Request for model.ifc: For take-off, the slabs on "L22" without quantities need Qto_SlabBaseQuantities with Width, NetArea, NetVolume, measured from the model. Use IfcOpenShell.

First a look at what the model holds.

```python
import ifcopenshell
import ifcopenshell.util.element
import ifcopenshell.util.unit

model = ifcopenshell.open("model.ifc")
print(model.schema)
for unit_type in ("LENGTHUNIT", "AREAUNIT", "VOLUMEUNIT"):
    print(unit_type, ifcopenshell.util.unit.calculate_unit_scale(model, unit_type))
storey = next(s for s in model.by_type("IfcBuildingStorey") if s.Name == "L22")
slabs = [e for e in ifcopenshell.util.element.get_decomposition(storey) if e.is_a("IfcSlab")]
for e in sorted(slabs, key=lambda e: e.id()):
    print(e.id(), e.is_a(), e.Name, list(ifcopenshell.util.element.get_psets(e, qtos_only=True)), sep=" | ")
```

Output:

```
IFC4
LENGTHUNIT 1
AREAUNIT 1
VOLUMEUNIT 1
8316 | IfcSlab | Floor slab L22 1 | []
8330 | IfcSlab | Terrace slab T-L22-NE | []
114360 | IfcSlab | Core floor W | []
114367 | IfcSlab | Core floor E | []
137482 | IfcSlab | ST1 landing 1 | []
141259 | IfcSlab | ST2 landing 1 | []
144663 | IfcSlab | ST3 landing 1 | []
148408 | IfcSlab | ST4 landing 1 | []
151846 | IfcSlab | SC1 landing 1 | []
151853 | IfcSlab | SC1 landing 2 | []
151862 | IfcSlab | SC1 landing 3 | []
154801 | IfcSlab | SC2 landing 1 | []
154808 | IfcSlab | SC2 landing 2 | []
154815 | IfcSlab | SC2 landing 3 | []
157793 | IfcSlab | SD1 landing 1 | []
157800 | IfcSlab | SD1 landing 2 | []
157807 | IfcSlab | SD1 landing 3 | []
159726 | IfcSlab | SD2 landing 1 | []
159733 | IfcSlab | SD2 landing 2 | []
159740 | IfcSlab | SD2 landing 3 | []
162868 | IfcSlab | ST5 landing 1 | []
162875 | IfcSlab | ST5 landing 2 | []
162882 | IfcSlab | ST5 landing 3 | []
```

```python
import ifcopenshell
import ifcopenshell.api.pset
import ifcopenshell.geom
import ifcopenshell.util.element
import ifcopenshell.util.shape
import ifcopenshell.util.unit

model = ifcopenshell.open("model.ifc")
unit_scale = ifcopenshell.util.unit.calculate_unit_scale(model)
area_scale = ifcopenshell.util.unit.calculate_unit_scale(model, "AREAUNIT")
volume_scale = ifcopenshell.util.unit.calculate_unit_scale(model, "VOLUMEUNIT")
settings = ifcopenshell.geom.settings()

storey = next(s for s in model.by_type("IfcBuildingStorey") if s.Name == "L22")
slabs = [e for e in ifcopenshell.util.element.get_decomposition(storey) if e.is_a("IfcSlab")]

for e in sorted(slabs, key=lambda e: e.id()):
    if ifcopenshell.util.element.get_psets(e, qtos_only=True, should_inherit=False):
        continue
    # Geometry comes back in metres, in the element's own axes.
    shape = ifcopenshell.geom.create_shape(settings, e)
    values = {
        "Width": ifcopenshell.util.shape.get_z(shape.geometry) / unit_scale,
        "NetArea": ifcopenshell.util.shape.get_footprint_area(shape.geometry) / area_scale,
        "NetVolume": ifcopenshell.util.shape.get_volume(shape.geometry) / volume_scale,
    }
    qto = ifcopenshell.api.pset.add_qto(model, product=e, name="Qto_SlabBaseQuantities")
    ifcopenshell.api.pset.edit_qto(model, qto=qto, properties=values)
    print(e.id(), {k: round(v, 3) for k, v in values.items()})

model.write("model_updated.ifc")
```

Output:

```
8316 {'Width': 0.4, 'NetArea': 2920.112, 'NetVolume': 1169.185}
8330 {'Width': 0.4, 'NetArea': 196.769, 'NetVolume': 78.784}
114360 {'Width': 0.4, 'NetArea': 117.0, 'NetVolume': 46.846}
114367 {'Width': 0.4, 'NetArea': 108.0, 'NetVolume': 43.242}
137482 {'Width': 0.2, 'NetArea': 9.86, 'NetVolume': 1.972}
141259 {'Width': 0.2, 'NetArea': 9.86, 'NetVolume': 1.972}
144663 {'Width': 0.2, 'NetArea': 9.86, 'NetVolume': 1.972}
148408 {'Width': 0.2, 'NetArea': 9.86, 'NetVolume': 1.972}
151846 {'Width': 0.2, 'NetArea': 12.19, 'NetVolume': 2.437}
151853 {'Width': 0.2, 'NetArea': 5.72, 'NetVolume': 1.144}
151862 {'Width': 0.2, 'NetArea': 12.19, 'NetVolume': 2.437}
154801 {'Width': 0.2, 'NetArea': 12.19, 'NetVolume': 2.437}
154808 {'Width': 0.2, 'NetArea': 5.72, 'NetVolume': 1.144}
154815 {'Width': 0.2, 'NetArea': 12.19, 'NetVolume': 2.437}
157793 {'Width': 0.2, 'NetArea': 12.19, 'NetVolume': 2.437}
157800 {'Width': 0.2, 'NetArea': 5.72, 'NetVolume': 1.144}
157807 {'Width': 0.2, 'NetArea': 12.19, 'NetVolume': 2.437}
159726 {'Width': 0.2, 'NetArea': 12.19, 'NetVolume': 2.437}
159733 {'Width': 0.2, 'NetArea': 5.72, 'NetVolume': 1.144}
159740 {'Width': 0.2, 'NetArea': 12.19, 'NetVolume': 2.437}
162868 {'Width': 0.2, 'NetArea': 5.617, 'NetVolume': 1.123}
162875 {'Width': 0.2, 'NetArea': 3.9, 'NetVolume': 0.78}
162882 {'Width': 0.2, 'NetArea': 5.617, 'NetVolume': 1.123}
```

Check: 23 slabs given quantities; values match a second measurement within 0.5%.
